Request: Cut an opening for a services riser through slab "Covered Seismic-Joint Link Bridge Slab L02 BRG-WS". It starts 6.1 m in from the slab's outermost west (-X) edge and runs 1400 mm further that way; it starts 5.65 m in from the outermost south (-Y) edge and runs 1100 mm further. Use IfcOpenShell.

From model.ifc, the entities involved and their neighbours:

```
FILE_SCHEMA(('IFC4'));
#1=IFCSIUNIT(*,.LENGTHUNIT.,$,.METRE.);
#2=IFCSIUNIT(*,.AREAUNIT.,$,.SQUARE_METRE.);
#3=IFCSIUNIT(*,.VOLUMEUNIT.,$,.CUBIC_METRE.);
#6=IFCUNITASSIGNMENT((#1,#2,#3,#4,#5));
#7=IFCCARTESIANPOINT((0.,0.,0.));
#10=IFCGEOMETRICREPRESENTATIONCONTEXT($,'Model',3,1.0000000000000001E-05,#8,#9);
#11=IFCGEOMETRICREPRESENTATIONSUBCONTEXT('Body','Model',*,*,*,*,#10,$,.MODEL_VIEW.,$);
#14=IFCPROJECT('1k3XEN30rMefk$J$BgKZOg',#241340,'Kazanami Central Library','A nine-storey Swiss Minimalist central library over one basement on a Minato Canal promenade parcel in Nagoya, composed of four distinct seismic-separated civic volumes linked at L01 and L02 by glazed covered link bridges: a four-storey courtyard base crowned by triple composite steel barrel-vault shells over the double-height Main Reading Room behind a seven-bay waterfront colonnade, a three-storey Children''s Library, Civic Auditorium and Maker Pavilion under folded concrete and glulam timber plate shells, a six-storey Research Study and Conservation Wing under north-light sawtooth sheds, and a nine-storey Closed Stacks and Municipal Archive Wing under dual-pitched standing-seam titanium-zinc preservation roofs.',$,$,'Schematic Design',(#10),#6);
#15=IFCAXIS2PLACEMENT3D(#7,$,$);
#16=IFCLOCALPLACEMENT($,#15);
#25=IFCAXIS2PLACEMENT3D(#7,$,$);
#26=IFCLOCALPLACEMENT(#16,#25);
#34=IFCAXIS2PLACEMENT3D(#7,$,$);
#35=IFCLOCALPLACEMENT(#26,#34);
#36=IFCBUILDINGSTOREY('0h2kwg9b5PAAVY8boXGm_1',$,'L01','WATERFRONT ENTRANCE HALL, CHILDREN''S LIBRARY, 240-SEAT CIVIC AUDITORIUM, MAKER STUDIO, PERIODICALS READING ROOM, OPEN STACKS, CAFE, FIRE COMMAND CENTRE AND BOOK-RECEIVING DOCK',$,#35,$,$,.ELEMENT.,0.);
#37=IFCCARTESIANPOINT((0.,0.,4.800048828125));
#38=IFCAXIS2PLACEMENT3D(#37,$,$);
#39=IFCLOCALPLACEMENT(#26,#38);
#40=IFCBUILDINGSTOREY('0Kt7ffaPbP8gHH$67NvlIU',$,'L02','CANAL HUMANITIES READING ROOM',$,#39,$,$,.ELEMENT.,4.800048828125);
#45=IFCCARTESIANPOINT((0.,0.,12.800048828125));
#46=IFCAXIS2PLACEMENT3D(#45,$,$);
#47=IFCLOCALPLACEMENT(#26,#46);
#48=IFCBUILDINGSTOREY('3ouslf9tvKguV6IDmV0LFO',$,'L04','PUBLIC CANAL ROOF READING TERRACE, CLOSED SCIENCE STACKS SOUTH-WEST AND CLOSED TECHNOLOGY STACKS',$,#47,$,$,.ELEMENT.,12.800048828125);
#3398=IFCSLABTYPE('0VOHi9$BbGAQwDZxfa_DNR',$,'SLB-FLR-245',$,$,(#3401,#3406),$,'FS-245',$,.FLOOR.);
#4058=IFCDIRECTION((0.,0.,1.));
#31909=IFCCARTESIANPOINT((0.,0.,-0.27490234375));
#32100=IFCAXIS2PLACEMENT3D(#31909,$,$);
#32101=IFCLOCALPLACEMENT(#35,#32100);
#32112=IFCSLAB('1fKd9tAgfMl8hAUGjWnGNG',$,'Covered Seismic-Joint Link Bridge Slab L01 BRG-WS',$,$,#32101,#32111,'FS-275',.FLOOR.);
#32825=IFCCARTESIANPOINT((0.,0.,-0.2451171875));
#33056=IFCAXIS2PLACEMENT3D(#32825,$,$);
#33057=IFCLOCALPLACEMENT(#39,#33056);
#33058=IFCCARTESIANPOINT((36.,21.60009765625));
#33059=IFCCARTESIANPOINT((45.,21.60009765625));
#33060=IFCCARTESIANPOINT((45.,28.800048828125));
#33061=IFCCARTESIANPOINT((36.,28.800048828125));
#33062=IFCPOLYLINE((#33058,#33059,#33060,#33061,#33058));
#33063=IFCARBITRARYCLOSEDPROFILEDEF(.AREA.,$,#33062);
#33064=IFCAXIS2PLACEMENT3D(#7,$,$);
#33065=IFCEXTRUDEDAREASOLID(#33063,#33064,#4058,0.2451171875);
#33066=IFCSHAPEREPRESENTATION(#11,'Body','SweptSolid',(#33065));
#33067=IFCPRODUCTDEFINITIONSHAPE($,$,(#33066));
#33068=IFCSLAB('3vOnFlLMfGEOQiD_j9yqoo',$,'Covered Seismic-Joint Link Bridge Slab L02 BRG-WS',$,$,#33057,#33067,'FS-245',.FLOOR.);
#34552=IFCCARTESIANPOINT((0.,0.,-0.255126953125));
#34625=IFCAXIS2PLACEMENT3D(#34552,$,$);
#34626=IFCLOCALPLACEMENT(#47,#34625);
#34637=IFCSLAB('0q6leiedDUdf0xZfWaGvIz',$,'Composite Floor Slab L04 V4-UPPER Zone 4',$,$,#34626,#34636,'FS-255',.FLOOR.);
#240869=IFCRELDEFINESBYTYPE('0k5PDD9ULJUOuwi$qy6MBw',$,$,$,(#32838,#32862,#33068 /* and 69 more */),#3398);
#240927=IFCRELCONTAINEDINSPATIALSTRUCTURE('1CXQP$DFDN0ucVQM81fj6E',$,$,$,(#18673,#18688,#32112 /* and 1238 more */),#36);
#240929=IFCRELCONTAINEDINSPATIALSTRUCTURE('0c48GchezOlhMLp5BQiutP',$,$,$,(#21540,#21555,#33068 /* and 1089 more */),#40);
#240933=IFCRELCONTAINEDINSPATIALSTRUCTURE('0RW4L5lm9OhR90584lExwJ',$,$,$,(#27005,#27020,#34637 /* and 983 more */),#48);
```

```python
import numpy as np
import ifcopenshell
import ifcopenshell.api.feature
import ifcopenshell.api.geometry
import ifcopenshell.api.root
import ifcopenshell.geom
import ifcopenshell.util.placement
import ifcopenshell.util.representation
import ifcopenshell.util.shape
import ifcopenshell.util.unit

model = ifcopenshell.open("model.ifc")
unit_scale = ifcopenshell.util.unit.calculate_unit_scale(model)
settings = ifcopenshell.geom.settings()


def volume(element):
    """Net volume in cubic metres, openings subtracted."""
    shape = ifcopenshell.geom.create_shape(settings, element)
    return ifcopenshell.util.shape.get_volume(shape.geometry)


slab = model.by_id(33068)
before = volume(slab)

# Extent in the slab's own axes, in metres. The edges named are its -X and -Y sides.
slab_shape = ifcopenshell.geom.create_shape(settings, slab)
vertices = ifcopenshell.util.shape.get_vertices(slab_shape.geometry)
x_min, y_min, bottom = vertices.min(axis=0)
top = vertices[:, 2].max()

opening = ifcopenshell.api.root.create_entity(model, ifc_class="IfcOpeningElement", name="Services riser opening", predefined_type="OPENING")
context = ifcopenshell.util.representation.get_context(model, "Model", "Body", "MODEL_VIEW")
width, depth = 1.4, 1.1
outline = [(0.0, 0.0), (width, 0.0), (width, depth), (0.0, depth), (0.0, 0.0)]
# Overshoot both faces by 50 mm so the cut is clean.
shape = ifcopenshell.api.geometry.add_slab_representation(
    model, context=context, depth=top - bottom + 0.1, polyline=outline
)
ifcopenshell.api.geometry.assign_representation(model, product=opening, representation=shape)

matrix = ifcopenshell.util.placement.get_local_placement(slab.ObjectPlacement)
matrix[:, 3] = matrix @ np.append(np.array([x_min + 6.1, y_min + 5.65, bottom - 0.05]) / unit_scale, 1.0)
ifcopenshell.api.geometry.edit_object_placement(model, product=opening, matrix=matrix, is_si=False)
ifcopenshell.api.feature.add_feature(model, feature=opening, element=slab)

after = volume(slab)

print(f"slab volume {before:.3f} -> {after:.3f} m3")

model.write("model_edited.ifc")
```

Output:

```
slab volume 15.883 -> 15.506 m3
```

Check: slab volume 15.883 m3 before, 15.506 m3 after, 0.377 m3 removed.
